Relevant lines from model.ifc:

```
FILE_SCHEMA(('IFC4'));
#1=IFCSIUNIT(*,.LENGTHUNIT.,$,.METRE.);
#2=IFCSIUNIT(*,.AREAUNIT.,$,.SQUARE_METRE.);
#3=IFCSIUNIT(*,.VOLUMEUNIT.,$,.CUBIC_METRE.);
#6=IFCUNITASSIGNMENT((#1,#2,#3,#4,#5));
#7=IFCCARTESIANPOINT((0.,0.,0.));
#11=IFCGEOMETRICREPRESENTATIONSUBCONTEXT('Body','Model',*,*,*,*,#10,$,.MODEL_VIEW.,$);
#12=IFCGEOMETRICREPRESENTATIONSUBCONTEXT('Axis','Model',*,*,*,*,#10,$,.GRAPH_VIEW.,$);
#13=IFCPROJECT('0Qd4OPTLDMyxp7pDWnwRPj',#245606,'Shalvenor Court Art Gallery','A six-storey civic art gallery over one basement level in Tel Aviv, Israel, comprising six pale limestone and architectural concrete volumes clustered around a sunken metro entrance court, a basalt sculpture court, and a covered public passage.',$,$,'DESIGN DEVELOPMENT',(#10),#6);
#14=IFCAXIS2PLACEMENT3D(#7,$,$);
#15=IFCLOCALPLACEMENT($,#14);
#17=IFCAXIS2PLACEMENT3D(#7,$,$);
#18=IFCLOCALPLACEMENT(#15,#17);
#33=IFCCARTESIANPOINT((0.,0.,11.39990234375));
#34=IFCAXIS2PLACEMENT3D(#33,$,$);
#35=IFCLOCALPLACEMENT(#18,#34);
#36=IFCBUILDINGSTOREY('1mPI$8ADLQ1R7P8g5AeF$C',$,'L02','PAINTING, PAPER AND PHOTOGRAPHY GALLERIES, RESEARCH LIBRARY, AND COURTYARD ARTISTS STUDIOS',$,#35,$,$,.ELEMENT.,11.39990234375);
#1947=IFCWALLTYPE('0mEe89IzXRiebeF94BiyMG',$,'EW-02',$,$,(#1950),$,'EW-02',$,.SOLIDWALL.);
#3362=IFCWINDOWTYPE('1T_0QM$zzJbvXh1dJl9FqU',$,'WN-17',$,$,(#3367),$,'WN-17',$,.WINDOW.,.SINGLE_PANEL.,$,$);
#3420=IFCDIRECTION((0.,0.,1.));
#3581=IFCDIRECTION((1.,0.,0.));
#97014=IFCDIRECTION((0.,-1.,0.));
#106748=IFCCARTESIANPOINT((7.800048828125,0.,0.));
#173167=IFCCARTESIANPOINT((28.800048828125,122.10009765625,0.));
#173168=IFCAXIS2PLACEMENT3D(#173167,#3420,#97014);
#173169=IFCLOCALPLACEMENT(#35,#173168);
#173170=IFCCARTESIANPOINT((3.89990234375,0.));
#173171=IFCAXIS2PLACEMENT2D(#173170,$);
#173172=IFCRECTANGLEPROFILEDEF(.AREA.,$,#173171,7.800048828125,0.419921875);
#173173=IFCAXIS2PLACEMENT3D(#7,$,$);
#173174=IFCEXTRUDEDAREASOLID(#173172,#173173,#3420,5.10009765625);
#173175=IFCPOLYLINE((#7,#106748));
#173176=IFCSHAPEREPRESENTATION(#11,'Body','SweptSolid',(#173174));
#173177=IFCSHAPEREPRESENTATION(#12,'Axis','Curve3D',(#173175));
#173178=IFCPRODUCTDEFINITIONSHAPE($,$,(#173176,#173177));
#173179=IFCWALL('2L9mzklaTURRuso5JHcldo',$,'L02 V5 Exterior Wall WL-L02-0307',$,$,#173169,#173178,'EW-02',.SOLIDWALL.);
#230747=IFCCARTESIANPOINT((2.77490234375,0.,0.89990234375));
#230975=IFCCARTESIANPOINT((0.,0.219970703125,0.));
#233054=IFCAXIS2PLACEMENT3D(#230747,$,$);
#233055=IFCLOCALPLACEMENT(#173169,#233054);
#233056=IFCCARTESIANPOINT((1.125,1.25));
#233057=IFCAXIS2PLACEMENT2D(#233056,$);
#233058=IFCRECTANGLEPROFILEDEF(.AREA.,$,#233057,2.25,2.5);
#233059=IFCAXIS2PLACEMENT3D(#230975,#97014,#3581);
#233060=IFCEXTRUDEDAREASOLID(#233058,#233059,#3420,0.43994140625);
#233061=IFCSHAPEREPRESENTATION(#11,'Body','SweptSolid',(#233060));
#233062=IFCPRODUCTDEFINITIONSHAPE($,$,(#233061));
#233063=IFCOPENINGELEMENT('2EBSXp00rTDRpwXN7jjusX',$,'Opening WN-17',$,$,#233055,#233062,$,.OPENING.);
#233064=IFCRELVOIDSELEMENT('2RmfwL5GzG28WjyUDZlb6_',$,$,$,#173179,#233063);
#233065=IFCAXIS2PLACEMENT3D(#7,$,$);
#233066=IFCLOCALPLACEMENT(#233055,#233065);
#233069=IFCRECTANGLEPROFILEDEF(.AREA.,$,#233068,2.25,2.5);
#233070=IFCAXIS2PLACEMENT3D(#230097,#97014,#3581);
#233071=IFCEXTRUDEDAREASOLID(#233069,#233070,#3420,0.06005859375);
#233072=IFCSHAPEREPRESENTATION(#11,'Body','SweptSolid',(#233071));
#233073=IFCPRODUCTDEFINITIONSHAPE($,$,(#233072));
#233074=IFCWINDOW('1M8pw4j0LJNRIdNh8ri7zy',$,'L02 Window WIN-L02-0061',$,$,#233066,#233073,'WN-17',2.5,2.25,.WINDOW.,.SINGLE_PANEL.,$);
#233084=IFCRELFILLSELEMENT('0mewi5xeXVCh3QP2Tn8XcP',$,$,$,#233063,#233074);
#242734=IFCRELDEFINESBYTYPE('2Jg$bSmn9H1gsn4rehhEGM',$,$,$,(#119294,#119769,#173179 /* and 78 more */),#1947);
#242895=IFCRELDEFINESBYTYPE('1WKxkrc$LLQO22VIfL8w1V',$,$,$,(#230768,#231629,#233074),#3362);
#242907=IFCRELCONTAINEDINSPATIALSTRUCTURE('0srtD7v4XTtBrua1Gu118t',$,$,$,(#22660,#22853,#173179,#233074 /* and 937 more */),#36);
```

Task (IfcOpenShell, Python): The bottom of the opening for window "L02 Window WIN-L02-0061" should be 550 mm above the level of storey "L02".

```python
import numpy as np
import ifcopenshell
import ifcopenshell.api.geometry
import ifcopenshell.geom
import ifcopenshell.util.element
import ifcopenshell.util.placement
import ifcopenshell.util.shape
import ifcopenshell.util.unit

model = ifcopenshell.open("model.ifc")
unit_scale = ifcopenshell.util.unit.calculate_unit_scale(model)

window = model.by_id(233074)
opening = window.FillsVoids[0].RelatingOpeningElement
storey = ifcopenshell.util.element.get_container(window, ifc_class="IfcBuildingStorey")
level = ifcopenshell.util.placement.get_local_placement(storey.ObjectPlacement)[2, 3]

# The opening's origin need not be at the sill, so measure its lowest point.
shape = ifcopenshell.geom.create_shape(ifcopenshell.geom.settings(), opening)
bottom = ifcopenshell.util.shape.get_shape_bottom_elevation(shape, shape.geometry) / unit_scale
dz = level + 0.55 / unit_scale - bottom

shift = np.array([0.0, 0.0, dz])
# The window is placed relative to its opening, so it follows when the opening moves.
matrix = ifcopenshell.util.placement.get_local_placement(opening.ObjectPlacement)
matrix[:3, 3] += shift
ifcopenshell.api.geometry.edit_object_placement(
    model, product=opening, matrix=matrix, is_si=False, should_transform_children=True
)

print(f"moved by {dz * unit_scale:+.3f} m")

model.write("model_updated.ifc")
```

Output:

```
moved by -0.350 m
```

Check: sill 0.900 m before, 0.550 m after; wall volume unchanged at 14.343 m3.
